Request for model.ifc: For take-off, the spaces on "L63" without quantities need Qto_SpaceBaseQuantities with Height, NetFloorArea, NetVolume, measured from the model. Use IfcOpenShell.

First a look at what the model holds.

```python
import ifcopenshell
import ifcopenshell.util.element
import ifcopenshell.util.unit

model = ifcopenshell.open("model.ifc")
print(model.schema)
for unit_type in ("LENGTHUNIT", "AREAUNIT", "VOLUMEUNIT"):
    print(unit_type, ifcopenshell.util.unit.calculate_unit_scale(model, unit_type))
storey = next(s for s in model.by_type("IfcBuildingStorey") if s.Name == "L63")
spaces = [e for e in ifcopenshell.util.element.get_decomposition(storey) if e.is_a("IfcSpace")]
for e in sorted(spaces, key=lambda e: e.id()):
    print(e.id(), e.is_a(), e.Name, list(ifcopenshell.util.element.get_psets(e, qtos_only=True)), sep=" | ")
```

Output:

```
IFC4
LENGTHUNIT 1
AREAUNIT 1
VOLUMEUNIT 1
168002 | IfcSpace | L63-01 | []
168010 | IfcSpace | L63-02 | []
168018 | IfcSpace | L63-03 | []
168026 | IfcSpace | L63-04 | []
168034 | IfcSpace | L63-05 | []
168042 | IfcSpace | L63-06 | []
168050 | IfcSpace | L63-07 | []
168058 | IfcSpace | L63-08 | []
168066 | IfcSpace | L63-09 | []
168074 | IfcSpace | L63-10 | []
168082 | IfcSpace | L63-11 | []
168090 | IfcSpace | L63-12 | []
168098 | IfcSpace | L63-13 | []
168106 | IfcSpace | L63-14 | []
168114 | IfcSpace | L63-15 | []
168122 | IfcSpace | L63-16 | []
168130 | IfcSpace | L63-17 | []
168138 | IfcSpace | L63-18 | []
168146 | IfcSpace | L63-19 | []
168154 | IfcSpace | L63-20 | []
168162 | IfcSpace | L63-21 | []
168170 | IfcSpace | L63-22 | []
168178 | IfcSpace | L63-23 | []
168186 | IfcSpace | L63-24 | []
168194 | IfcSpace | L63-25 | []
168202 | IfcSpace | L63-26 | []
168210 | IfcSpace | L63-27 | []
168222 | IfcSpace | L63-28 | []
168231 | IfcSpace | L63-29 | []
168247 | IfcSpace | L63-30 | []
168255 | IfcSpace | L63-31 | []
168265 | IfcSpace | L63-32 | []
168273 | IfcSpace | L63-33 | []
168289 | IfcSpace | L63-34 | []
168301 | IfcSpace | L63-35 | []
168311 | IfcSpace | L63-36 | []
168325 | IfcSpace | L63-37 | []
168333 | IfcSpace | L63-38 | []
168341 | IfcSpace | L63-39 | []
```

```python
import ifcopenshell
import ifcopenshell.api.pset
import ifcopenshell.geom
import ifcopenshell.util.element
import ifcopenshell.util.shape
import ifcopenshell.util.unit

model = ifcopenshell.open("model.ifc")
unit_scale = ifcopenshell.util.unit.calculate_unit_scale(model)
area_scale = ifcopenshell.util.unit.calculate_unit_scale(model, "AREAUNIT")
volume_scale = ifcopenshell.util.unit.calculate_unit_scale(model, "VOLUMEUNIT")
settings = ifcopenshell.geom.settings()

storey = next(s for s in model.by_type("IfcBuildingStorey") if s.Name == "L63")
spaces = [e for e in ifcopenshell.util.element.get_decomposition(storey) if e.is_a("IfcSpace")]

for e in sorted(spaces, key=lambda e: e.id()):
    if ifcopenshell.util.element.get_psets(e, qtos_only=True, should_inherit=False):
        continue
    # Geometry comes back in metres, in the element's own axes.
    shape = ifcopenshell.geom.create_shape(settings, e)
    values = {
        "Height": ifcopenshell.util.shape.get_z(shape.geometry) / unit_scale,
        "NetFloorArea": ifcopenshell.util.shape.get_footprint_area(shape.geometry) / area_scale,
        "NetVolume": ifcopenshell.util.shape.get_volume(shape.geometry) / volume_scale,
    }
    qto = ifcopenshell.api.pset.add_qto(model, product=e, name="Qto_SpaceBaseQuantities")
    ifcopenshell.api.pset.edit_qto(model, qto=qto, properties=values)
    print(e.id(), {k: round(v, 3) for k, v in values.items()})

model.write("model_updated.ifc")
```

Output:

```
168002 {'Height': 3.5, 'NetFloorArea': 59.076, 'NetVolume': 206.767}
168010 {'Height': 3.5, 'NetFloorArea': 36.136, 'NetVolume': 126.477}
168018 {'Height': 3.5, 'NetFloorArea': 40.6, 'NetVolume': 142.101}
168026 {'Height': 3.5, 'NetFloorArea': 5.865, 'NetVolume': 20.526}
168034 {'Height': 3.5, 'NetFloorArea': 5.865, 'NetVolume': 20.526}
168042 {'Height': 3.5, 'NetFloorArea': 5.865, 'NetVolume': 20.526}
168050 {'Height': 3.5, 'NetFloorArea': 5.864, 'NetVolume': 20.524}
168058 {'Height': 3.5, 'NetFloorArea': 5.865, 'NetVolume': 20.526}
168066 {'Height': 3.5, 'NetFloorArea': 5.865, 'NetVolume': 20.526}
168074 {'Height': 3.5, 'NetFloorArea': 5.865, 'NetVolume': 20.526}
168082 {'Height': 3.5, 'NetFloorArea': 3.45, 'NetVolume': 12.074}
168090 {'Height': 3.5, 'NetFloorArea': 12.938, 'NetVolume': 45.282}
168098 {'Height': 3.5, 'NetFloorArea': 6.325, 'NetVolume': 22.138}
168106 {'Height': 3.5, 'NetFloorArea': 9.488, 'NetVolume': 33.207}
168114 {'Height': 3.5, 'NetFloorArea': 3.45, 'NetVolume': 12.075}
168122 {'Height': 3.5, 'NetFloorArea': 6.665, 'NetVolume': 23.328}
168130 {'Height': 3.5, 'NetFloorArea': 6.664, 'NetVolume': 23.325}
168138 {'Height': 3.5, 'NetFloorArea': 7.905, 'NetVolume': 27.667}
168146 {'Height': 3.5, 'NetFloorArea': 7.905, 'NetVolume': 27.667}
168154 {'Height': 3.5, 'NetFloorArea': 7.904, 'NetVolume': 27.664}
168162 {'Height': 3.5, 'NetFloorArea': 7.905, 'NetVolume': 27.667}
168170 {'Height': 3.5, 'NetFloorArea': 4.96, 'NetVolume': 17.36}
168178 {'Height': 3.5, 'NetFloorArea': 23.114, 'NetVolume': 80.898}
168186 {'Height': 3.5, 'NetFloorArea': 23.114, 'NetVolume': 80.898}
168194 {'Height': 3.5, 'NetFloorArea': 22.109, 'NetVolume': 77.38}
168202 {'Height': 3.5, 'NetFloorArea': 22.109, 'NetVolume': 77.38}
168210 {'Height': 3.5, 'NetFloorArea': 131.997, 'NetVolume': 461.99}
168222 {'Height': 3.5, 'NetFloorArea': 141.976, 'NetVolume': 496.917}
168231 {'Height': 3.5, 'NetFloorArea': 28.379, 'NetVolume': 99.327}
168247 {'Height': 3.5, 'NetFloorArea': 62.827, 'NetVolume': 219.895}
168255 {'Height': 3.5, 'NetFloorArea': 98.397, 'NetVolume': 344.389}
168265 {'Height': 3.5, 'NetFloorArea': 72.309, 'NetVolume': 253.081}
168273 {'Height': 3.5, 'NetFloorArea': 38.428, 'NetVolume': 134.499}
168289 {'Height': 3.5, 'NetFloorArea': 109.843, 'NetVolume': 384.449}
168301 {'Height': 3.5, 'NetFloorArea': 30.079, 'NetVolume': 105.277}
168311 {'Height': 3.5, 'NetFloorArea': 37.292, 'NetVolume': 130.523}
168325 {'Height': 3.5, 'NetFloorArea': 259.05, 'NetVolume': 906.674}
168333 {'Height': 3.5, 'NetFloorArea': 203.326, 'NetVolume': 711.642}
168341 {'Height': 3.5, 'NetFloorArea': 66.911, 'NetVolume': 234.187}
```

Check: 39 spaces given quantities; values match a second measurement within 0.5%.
